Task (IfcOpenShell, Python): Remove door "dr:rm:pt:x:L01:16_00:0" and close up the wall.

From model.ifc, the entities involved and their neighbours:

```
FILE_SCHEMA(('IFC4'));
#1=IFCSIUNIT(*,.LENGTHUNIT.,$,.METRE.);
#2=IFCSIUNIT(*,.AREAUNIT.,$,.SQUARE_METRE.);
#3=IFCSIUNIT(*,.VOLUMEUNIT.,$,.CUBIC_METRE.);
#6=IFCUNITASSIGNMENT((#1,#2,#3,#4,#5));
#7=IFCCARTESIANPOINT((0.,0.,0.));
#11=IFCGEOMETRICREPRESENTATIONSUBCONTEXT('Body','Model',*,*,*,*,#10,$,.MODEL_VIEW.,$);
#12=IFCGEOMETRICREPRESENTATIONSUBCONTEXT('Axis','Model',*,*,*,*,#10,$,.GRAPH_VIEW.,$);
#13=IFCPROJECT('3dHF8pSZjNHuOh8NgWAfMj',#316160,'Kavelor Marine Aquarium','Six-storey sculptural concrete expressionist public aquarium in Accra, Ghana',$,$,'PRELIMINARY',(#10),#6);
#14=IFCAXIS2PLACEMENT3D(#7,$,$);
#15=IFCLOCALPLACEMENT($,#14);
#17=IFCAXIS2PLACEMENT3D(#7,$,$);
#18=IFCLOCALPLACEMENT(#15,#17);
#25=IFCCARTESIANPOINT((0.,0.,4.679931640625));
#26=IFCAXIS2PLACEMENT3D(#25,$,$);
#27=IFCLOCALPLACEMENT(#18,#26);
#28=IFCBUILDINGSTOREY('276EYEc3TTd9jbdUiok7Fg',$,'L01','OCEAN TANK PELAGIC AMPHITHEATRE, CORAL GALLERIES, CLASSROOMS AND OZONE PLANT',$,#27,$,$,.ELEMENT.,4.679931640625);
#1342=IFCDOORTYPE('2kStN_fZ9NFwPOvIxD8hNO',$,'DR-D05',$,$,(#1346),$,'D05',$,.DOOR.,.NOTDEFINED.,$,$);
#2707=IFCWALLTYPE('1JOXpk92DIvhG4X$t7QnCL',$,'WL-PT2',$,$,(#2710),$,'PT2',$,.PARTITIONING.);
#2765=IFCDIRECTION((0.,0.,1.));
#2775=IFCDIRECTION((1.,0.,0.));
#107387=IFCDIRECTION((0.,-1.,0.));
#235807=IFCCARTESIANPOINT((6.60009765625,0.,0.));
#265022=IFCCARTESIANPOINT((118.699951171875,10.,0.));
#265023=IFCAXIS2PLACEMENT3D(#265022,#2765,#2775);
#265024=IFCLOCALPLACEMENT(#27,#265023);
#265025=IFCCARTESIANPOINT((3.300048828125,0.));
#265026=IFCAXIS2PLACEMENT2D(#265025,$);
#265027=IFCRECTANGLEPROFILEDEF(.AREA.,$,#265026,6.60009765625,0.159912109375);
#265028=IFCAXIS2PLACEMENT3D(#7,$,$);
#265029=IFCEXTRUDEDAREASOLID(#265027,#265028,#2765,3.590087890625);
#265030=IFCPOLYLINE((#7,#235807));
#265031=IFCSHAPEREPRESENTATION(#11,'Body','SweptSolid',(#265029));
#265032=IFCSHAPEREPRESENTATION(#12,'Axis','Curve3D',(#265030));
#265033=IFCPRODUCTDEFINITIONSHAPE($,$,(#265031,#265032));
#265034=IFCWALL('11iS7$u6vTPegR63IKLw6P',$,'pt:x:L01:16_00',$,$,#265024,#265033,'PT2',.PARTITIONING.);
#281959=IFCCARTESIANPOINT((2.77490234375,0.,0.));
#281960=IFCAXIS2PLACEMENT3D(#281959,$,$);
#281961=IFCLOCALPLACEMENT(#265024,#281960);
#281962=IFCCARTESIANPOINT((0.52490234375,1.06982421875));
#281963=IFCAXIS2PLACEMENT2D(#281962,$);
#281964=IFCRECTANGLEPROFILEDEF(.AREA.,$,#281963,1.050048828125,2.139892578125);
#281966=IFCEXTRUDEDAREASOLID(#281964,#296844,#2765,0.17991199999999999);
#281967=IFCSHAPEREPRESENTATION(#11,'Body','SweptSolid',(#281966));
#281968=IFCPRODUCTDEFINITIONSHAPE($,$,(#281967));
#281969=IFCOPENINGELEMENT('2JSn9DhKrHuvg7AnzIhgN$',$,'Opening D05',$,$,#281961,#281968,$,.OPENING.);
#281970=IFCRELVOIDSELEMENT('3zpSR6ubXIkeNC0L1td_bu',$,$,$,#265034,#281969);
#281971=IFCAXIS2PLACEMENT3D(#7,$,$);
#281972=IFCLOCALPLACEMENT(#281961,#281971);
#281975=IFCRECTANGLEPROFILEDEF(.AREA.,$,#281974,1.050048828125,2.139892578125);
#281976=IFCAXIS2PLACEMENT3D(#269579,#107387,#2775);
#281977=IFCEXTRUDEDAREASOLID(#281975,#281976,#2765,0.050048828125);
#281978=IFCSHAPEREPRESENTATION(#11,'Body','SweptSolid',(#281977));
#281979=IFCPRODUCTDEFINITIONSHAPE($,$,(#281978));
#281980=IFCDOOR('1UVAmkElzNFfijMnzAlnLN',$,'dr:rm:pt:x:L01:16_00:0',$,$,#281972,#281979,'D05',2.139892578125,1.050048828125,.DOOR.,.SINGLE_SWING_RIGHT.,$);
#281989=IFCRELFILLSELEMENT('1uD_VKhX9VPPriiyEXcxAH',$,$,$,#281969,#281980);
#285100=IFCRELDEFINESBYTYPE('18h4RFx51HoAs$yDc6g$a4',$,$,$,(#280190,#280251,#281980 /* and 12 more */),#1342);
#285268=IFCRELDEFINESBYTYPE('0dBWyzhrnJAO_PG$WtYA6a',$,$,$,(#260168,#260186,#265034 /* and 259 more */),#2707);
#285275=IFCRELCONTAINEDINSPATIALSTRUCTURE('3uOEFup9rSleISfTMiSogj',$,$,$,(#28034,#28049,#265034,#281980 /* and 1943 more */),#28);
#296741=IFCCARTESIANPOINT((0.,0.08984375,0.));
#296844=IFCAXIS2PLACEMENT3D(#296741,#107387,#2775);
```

```python
import ifcopenshell
import ifcopenshell.api.feature
import ifcopenshell.api.root
import ifcopenshell.geom
import ifcopenshell.util.shape

model = ifcopenshell.open("model.ifc")
settings = ifcopenshell.geom.settings()


def volume(element):
    """Net volume in cubic metres, openings subtracted."""
    shape = ifcopenshell.geom.create_shape(settings, element)
    return ifcopenshell.util.shape.get_volume(shape.geometry)


door = model.by_guid("1UVAmkElzNFfijMnzAlnLN")
opening = door.FillsVoids[0].RelatingOpeningElement
wall = opening.VoidsElements[0].RelatingBuildingElement
before = volume(wall)

ifcopenshell.api.root.remove_product(model, product=door)
ifcopenshell.api.feature.remove_feature(model, feature=opening)

after = volume(wall)

print(f"wall volume {before:.3f} -> {after:.3f} m3")

model.write("model_edited.ifc")
```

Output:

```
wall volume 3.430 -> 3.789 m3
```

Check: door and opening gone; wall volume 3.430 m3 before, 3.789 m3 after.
